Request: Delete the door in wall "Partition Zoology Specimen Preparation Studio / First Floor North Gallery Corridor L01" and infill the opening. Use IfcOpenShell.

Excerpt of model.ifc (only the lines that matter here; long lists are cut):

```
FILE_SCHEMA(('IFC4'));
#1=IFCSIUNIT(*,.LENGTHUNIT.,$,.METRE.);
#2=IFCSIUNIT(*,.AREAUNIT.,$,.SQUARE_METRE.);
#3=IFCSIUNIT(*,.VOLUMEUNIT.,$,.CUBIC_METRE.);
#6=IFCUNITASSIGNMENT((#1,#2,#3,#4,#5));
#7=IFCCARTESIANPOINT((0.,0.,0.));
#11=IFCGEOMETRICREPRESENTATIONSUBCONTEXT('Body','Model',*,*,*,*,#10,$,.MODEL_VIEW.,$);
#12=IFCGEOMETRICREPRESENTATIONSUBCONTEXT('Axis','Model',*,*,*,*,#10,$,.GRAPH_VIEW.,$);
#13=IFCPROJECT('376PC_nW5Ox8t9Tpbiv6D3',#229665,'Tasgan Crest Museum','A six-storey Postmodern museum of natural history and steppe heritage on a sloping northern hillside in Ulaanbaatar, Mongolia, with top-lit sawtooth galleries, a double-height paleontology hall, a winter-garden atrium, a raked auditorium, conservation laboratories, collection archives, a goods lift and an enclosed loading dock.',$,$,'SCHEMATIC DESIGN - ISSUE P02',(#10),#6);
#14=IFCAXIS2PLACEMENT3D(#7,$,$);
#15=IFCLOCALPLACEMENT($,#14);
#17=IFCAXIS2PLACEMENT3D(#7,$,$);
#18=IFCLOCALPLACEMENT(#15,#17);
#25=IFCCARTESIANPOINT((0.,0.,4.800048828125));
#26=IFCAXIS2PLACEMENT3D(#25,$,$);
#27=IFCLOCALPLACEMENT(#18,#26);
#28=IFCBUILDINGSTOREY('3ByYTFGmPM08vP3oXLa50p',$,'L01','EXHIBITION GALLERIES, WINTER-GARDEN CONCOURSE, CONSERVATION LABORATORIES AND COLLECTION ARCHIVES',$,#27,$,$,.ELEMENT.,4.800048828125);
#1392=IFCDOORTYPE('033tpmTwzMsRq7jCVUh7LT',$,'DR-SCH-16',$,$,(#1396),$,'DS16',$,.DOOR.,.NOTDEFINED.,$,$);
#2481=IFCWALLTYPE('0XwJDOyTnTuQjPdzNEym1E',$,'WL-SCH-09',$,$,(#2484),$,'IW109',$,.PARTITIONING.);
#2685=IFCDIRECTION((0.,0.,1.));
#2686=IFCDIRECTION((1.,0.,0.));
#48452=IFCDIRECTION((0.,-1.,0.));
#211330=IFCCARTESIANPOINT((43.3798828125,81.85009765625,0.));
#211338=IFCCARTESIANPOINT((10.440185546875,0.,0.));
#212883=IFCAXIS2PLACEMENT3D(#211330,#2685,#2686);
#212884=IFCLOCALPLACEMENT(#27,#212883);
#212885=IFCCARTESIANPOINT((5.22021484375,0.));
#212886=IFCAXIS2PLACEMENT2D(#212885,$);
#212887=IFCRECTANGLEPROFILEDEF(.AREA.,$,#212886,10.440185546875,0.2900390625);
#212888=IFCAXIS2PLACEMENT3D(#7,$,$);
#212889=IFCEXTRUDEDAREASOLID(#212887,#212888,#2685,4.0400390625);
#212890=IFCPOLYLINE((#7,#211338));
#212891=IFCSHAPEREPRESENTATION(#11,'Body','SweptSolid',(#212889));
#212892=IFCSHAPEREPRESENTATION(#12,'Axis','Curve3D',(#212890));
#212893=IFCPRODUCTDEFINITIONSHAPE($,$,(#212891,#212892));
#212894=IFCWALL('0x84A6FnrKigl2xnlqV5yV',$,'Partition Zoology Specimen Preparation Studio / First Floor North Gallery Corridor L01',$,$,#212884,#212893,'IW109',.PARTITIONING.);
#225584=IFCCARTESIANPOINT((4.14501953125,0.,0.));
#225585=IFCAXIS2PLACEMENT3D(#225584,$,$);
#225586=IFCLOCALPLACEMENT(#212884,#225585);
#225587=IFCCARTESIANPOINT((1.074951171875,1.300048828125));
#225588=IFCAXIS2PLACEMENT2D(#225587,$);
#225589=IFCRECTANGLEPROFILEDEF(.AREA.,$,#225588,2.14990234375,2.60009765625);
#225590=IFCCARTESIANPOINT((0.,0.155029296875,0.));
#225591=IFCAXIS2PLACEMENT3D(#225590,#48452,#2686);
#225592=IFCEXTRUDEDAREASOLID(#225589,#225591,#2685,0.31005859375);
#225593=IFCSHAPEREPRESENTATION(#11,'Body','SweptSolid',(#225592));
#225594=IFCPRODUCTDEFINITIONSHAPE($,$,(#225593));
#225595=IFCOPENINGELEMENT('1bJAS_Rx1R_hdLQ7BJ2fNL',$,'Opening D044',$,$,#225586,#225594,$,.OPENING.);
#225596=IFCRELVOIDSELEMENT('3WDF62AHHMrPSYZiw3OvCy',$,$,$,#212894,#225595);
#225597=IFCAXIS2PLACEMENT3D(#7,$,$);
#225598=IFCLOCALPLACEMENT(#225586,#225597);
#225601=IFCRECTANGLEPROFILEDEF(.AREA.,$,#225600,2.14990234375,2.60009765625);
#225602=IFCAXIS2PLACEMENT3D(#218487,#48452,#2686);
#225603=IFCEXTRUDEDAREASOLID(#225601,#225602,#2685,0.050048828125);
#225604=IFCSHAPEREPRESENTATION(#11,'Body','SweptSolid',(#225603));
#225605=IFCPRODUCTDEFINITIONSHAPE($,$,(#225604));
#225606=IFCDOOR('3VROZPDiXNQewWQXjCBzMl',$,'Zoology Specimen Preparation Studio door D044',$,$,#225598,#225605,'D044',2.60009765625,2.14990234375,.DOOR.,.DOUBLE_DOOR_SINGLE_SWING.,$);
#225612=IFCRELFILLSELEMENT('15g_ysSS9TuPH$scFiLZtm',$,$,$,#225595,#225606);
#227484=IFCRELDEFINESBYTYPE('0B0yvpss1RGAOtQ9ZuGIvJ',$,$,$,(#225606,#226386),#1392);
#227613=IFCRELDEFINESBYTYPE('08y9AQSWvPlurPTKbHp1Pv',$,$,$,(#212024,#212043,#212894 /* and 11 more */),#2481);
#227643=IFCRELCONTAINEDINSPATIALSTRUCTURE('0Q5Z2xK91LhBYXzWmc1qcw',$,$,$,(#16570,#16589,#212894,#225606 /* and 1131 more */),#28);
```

```python
import ifcopenshell
import ifcopenshell.api.feature
import ifcopenshell.api.root
import ifcopenshell.geom
import ifcopenshell.util.shape

model = ifcopenshell.open("model.ifc")
settings = ifcopenshell.geom.settings()


def volume(element):
    """Net volume in cubic metres, openings subtracted."""
    shape = ifcopenshell.geom.create_shape(settings, element)
    return ifcopenshell.util.shape.get_volume(shape.geometry)


door = model.by_guid("3VROZPDiXNQewWQXjCBzMl")
opening = door.FillsVoids[0].RelatingOpeningElement
wall = opening.VoidsElements[0].RelatingBuildingElement
before = volume(wall)

ifcopenshell.api.root.remove_product(model, product=door)
ifcopenshell.api.feature.remove_feature(model, feature=opening)

after = volume(wall)

print(f"wall volume {before:.3f} -> {after:.3f} m3")

model.write("model_rev.ifc")
```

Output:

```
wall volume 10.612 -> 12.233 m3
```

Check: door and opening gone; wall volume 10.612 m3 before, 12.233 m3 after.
